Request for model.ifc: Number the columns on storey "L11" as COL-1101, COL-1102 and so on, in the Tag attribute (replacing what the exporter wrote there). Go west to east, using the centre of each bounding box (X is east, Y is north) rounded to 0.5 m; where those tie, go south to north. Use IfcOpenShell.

First a look at what the model holds.

```python
import ifcopenshell
import ifcopenshell.util.element
import ifcopenshell.util.placement

model = ifcopenshell.open("model.ifc")
print(model.schema)
storey = next(s for s in model.by_type("IfcBuildingStorey") if s.Name == "L11")
columns = [e for e in ifcopenshell.util.element.get_decomposition(storey) if e.is_a("IfcColumn")]
for e in sorted(columns, key=lambda e: e.id()):
    origin = ifcopenshell.util.placement.get_local_placement(e.ObjectPlacement)[:3, 3]
    print(e.id(), e.Tag, e.Name, origin.round(2) + 0.0, sep=" | ")
```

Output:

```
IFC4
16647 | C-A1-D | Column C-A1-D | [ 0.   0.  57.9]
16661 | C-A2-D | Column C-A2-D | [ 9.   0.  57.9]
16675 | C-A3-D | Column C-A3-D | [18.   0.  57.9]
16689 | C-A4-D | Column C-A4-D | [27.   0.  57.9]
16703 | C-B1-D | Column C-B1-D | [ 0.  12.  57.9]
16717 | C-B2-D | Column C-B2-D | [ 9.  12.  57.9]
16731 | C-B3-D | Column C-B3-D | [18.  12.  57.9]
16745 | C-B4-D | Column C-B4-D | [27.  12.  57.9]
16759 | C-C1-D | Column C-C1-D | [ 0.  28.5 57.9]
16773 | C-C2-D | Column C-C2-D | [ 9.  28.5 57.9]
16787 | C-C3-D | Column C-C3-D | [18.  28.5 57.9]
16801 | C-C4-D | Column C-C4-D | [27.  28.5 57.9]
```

```python
import ifcopenshell
import ifcopenshell.geom
import ifcopenshell.util.element
import ifcopenshell.util.shape

model = ifcopenshell.open("model.ifc")
settings = ifcopenshell.geom.settings()
settings.set("use-world-coords", True)


def centre(element):
    shape = ifcopenshell.geom.create_shape(settings, element)
    return ifcopenshell.util.shape.get_bbox_centroid(shape.geometry)


storey = next(s for s in model.by_type("IfcBuildingStorey") if s.Name == "L11")
columns = [e for e in ifcopenshell.util.element.get_decomposition(storey) if e.is_a("IfcColumn")]

# Insertion points can sit at a corner or the storey origin, so sort by the geometry (in metres).
centres = {e: centre(e) for e in columns}
columns.sort(key=lambda e: (round(centres[e][0] / 0.5), centres[e][1]))

for i, e in enumerate(columns, start=1):
    number = f"COL-11{i:02d}"
    e.Tag = number
    print(e.id(), number)

model.write("model_rev.ifc")
```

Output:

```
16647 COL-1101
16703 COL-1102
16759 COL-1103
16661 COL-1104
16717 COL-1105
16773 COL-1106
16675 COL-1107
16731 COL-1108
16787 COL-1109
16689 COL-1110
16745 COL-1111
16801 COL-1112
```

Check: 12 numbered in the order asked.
